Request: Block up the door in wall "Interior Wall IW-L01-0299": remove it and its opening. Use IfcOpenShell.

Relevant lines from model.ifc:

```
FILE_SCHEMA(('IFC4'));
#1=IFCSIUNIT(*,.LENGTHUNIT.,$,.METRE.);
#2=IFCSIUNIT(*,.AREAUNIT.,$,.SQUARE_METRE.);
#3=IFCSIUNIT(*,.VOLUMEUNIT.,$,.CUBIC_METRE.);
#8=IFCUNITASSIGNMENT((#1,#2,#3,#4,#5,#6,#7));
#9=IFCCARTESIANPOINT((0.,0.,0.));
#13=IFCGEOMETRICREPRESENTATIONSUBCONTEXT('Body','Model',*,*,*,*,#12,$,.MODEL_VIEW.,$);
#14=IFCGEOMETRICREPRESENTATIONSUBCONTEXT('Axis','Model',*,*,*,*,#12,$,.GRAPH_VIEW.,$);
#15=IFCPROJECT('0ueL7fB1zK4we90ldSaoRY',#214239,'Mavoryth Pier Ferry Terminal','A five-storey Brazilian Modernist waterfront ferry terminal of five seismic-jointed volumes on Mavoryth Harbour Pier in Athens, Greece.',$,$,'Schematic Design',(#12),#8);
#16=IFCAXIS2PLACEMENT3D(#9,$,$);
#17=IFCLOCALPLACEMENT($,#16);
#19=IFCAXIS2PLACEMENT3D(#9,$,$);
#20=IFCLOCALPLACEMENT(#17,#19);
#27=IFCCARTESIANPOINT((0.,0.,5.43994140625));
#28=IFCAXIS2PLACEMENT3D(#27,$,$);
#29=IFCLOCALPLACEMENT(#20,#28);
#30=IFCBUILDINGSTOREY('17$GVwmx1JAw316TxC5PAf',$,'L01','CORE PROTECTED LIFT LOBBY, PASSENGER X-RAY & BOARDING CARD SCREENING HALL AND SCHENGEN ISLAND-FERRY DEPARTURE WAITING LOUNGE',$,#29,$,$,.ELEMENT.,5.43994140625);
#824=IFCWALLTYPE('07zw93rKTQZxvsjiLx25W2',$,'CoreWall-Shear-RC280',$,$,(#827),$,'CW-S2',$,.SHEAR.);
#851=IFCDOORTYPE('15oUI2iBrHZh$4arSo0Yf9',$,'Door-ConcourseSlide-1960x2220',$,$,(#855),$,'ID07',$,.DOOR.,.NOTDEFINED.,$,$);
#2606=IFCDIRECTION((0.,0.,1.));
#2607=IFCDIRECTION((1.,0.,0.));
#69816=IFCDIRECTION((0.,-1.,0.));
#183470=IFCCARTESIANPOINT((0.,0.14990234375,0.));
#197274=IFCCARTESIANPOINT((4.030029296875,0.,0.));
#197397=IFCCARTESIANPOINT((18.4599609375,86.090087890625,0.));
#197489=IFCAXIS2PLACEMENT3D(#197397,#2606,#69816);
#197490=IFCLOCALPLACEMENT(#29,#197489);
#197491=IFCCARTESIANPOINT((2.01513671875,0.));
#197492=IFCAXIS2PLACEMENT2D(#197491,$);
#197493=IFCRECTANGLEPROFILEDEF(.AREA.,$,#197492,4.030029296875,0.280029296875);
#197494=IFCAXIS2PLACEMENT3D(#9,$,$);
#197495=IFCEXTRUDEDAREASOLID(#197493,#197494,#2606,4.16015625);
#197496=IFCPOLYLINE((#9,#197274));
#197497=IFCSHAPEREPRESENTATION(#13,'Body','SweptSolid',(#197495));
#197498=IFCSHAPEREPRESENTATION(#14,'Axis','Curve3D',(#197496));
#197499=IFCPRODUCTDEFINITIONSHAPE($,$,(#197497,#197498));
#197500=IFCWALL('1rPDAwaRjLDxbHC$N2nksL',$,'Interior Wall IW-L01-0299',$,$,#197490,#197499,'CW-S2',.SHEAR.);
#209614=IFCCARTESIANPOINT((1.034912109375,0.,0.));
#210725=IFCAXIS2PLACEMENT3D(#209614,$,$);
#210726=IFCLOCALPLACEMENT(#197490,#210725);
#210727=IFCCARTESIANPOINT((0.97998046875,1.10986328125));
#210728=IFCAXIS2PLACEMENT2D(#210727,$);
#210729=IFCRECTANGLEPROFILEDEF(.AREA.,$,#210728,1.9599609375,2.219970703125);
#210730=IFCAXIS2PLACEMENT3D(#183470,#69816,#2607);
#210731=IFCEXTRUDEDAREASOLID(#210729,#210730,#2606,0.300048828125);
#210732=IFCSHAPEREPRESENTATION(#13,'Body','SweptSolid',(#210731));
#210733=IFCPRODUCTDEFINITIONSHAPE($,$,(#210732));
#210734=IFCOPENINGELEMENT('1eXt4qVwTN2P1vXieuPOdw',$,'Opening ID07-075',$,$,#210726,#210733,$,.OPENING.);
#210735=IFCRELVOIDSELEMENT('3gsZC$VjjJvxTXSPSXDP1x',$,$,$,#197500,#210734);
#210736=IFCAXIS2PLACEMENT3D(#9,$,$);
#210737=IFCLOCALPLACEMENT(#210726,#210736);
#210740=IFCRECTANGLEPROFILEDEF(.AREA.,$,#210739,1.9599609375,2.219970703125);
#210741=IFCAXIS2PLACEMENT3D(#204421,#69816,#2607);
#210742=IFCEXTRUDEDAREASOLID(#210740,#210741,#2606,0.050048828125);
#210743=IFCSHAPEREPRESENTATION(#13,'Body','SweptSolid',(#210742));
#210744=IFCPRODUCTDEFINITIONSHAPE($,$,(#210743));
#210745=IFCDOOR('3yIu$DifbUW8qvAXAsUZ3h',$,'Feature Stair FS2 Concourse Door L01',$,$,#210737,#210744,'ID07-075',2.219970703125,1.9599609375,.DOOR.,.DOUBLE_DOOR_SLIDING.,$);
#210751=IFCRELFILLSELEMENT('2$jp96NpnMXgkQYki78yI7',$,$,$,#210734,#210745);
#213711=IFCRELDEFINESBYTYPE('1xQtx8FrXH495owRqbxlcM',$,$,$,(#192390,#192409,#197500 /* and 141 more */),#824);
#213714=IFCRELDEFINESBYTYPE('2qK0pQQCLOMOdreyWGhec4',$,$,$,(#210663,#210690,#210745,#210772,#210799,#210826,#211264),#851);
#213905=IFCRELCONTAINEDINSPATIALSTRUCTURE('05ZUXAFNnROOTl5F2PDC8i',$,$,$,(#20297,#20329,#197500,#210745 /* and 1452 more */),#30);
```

```python
import ifcopenshell
import ifcopenshell.api.feature
import ifcopenshell.api.root
import ifcopenshell.geom
import ifcopenshell.util.shape

model = ifcopenshell.open("model.ifc")
settings = ifcopenshell.geom.settings()


def volume(element):
    """Net volume in cubic metres, openings subtracted."""
    shape = ifcopenshell.geom.create_shape(settings, element)
    return ifcopenshell.util.shape.get_volume(shape.geometry)


door = model.by_id(210745)
opening = door.FillsVoids[0].RelatingOpeningElement
wall = opening.VoidsElements[0].RelatingBuildingElement
before = volume(wall)

ifcopenshell.api.root.remove_product(model, product=door)
ifcopenshell.api.feature.remove_feature(model, feature=opening)

after = volume(wall)

print(f"wall volume {before:.3f} -> {after:.3f} m3")

model.write("model_rev.ifc")
```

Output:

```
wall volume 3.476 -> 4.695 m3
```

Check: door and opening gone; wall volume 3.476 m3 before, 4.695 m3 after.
